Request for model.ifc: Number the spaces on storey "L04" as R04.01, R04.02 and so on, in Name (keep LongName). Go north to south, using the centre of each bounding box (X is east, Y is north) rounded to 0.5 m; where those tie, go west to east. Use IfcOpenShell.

First a look at what the model holds.

```python
import ifcopenshell
import ifcopenshell.util.element
import ifcopenshell.util.placement

model = ifcopenshell.open("model.ifc")
print(model.schema)
storey = next(s for s in model.by_type("IfcBuildingStorey") if s.Name == "L04")
spaces = [e for e in ifcopenshell.util.element.get_decomposition(storey) if e.is_a("IfcSpace")]
for e in sorted(spaces, key=lambda e: e.id()):
    origin = ifcopenshell.util.placement.get_local_placement(e.ObjectPlacement)[:3, 3]
    print(e.id(), e.Name, e.LongName, origin.round(2) + 0.0, sep=" | ")
```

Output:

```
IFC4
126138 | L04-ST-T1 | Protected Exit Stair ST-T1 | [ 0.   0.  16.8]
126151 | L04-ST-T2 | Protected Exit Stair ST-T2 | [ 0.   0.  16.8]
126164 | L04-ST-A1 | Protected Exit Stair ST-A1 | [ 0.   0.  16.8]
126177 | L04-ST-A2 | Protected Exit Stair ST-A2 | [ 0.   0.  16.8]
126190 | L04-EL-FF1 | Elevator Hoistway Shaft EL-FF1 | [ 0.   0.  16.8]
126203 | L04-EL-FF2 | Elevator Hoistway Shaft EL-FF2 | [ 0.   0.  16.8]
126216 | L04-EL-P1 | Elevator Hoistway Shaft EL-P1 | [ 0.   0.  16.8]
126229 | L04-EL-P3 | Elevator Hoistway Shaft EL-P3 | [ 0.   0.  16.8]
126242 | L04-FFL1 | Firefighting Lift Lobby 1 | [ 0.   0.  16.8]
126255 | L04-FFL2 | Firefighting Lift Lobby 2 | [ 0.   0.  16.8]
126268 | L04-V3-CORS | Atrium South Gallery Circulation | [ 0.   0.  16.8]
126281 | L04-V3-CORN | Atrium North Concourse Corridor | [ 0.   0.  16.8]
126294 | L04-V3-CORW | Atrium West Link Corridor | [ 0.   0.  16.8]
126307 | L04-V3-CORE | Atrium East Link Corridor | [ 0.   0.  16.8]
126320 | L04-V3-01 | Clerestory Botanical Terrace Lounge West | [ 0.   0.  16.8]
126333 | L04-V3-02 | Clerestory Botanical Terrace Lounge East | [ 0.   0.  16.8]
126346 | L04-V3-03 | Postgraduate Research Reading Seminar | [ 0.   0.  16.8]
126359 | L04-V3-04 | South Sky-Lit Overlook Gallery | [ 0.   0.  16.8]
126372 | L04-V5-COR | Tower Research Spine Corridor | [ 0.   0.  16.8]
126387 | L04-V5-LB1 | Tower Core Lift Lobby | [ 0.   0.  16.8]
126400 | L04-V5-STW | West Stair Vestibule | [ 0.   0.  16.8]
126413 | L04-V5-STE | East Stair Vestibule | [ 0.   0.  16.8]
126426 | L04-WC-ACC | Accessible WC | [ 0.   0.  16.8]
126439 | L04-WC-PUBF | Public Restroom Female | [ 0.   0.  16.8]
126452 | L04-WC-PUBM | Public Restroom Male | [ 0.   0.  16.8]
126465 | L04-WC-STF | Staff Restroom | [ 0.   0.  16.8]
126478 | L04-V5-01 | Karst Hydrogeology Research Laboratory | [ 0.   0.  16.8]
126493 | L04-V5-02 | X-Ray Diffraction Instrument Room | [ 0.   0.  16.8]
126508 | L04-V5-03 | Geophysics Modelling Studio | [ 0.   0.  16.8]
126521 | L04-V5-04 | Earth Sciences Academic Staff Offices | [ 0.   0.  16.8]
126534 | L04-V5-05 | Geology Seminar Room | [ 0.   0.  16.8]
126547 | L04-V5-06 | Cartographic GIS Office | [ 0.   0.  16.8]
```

```python
import ifcopenshell
import ifcopenshell.geom
import ifcopenshell.util.element
import ifcopenshell.util.shape

model = ifcopenshell.open("model.ifc")
settings = ifcopenshell.geom.settings()
settings.set("use-world-coords", True)


def centre(element):
    shape = ifcopenshell.geom.create_shape(settings, element)
    return ifcopenshell.util.shape.get_bbox_centroid(shape.geometry)


storey = next(s for s in model.by_type("IfcBuildingStorey") if s.Name == "L04")
spaces = [e for e in ifcopenshell.util.element.get_decomposition(storey) if e.is_a("IfcSpace")]

# Insertion points can sit at a corner or the storey origin, so sort by the geometry (in metres).
centres = {e: centre(e) for e in spaces}
spaces.sort(key=lambda e: (-round(centres[e][1] / 0.5), centres[e][0]))

for i, e in enumerate(spaces, start=1):
    number = f"R04.{i:02d}"
    e.Name = number
    print(e.id(), number)

model.write("model_edited.ifc")
```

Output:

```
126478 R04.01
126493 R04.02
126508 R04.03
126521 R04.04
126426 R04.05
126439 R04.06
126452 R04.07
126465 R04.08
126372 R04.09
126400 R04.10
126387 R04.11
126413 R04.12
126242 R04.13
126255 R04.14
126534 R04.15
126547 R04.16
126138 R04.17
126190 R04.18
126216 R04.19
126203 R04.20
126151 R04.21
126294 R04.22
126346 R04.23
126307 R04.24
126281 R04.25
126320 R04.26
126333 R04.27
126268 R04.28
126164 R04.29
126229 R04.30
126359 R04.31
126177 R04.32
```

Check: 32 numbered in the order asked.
